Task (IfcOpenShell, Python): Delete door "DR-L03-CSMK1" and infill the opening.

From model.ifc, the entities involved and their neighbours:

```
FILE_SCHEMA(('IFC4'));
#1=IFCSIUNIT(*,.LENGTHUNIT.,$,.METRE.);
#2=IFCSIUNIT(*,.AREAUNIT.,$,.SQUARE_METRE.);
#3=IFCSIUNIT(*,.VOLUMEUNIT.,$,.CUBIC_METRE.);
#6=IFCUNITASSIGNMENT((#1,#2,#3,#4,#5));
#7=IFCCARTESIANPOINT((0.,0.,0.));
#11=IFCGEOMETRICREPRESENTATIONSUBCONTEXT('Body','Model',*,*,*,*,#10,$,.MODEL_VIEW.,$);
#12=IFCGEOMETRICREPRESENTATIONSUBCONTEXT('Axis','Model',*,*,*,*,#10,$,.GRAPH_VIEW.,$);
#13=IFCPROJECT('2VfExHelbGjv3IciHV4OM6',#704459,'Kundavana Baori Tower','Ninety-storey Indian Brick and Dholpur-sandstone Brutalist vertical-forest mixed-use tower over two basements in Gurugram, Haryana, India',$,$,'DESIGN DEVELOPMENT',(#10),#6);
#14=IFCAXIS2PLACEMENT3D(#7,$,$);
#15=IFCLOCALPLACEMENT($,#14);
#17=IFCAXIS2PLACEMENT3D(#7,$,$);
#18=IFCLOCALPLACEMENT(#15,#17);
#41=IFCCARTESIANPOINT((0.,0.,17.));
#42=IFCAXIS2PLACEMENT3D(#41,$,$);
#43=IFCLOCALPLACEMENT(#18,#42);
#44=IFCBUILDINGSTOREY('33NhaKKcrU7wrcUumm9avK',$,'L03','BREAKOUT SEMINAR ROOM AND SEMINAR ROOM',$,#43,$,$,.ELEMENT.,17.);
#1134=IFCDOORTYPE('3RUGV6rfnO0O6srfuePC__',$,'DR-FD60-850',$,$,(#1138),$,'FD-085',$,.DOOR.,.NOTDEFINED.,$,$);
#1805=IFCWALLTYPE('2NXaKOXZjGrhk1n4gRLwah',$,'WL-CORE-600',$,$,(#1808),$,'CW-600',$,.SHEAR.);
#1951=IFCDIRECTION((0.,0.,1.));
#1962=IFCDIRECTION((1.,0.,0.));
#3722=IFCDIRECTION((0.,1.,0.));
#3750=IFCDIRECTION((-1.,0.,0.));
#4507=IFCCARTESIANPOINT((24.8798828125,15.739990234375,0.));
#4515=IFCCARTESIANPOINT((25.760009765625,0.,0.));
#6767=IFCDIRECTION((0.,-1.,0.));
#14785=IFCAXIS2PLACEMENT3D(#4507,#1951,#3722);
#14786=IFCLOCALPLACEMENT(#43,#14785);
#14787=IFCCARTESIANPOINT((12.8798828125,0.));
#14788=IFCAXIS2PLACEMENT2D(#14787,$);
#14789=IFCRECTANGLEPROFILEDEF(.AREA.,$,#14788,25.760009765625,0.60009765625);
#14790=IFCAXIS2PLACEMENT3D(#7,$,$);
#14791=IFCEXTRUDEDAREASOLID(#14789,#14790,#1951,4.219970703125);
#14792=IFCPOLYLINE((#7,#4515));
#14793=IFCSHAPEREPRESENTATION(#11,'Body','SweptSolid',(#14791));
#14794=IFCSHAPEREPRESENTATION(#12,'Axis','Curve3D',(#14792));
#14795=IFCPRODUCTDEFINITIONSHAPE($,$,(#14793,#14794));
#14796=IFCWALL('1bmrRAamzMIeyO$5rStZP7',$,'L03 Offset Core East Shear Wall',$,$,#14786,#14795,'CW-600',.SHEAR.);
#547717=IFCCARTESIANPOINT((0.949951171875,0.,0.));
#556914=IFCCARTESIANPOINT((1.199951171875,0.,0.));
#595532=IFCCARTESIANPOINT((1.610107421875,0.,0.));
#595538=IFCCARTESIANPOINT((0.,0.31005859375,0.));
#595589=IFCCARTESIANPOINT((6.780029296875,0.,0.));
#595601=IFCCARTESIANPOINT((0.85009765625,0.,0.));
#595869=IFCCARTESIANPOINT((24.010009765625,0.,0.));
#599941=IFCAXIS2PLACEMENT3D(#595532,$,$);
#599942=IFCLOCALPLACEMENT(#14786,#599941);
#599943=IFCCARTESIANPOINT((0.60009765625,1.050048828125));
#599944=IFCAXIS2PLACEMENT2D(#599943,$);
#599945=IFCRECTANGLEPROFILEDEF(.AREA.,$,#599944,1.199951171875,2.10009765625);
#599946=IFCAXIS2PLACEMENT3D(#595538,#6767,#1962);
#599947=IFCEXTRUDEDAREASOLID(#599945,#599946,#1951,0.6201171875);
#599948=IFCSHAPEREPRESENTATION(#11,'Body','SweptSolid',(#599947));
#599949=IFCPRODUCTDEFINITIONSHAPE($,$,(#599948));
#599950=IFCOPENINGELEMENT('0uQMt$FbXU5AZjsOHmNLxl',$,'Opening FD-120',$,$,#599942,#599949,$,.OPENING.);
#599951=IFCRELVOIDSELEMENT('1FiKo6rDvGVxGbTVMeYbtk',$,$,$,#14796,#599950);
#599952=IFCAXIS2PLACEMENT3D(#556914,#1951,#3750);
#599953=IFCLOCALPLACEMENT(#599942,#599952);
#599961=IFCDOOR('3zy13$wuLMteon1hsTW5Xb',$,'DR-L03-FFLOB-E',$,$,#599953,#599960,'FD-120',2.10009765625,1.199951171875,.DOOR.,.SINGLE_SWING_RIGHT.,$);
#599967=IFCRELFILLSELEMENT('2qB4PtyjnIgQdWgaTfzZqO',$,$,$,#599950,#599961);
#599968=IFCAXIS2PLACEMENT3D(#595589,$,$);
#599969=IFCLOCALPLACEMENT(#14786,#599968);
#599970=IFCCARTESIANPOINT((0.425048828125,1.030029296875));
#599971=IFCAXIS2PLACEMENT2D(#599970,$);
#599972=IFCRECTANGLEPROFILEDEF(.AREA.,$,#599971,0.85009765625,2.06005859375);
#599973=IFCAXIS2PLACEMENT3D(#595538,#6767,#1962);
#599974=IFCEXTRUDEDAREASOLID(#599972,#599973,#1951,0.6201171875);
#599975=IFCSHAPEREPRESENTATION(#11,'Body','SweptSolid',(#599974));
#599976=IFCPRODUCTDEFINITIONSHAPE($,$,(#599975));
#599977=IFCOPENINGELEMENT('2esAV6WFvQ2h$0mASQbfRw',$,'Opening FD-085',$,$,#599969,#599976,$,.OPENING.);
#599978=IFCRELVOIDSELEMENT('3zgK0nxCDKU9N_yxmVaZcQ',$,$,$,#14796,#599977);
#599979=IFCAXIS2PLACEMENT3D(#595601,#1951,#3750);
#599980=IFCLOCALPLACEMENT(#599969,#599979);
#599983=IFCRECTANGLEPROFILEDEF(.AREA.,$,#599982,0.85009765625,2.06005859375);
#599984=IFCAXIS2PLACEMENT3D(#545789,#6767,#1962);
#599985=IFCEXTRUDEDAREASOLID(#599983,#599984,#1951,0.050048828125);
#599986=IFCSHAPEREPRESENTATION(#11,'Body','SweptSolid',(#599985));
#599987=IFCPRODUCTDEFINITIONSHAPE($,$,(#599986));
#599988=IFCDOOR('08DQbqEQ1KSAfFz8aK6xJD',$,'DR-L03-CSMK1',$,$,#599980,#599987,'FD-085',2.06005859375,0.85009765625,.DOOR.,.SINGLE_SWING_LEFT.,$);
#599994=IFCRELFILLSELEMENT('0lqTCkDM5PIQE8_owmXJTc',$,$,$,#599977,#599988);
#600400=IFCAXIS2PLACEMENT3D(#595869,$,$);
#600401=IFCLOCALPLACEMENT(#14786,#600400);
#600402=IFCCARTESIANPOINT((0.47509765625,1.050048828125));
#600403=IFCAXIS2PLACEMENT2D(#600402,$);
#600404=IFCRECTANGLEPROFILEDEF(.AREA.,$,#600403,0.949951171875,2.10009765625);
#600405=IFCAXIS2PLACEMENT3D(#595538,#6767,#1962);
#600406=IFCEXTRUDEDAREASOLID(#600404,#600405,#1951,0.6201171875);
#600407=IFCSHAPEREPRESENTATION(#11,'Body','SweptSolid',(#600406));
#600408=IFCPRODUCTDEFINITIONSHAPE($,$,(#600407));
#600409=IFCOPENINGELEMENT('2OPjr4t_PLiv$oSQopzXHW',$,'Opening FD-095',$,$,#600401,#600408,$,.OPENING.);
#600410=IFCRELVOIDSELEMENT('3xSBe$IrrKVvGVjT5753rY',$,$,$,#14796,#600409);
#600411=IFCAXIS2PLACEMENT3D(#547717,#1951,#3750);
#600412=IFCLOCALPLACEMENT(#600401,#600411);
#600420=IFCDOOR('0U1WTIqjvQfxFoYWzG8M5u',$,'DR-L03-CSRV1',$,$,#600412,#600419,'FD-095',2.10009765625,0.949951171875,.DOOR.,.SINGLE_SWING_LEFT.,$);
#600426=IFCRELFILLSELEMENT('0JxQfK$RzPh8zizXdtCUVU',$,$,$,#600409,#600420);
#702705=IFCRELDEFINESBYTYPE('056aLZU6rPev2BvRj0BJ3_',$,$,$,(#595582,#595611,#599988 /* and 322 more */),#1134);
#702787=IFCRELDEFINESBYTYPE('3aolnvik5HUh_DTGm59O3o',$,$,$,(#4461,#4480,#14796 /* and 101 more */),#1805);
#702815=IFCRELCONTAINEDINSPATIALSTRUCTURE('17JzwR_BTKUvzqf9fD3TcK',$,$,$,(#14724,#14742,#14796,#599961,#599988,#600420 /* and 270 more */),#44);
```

```python
import ifcopenshell
import ifcopenshell.api.feature
import ifcopenshell.api.root
import ifcopenshell.geom
import ifcopenshell.util.shape

model = ifcopenshell.open("model.ifc")
settings = ifcopenshell.geom.settings()


def volume(element):
    """Net volume in cubic metres, openings subtracted."""
    shape = ifcopenshell.geom.create_shape(settings, element)
    return ifcopenshell.util.shape.get_volume(shape.geometry)


door = model.by_guid("08DQbqEQ1KSAfFz8aK6xJD")
opening = door.FillsVoids[0].RelatingOpeningElement
wall = opening.VoidsElements[0].RelatingBuildingElement
before = volume(wall)

ifcopenshell.api.root.remove_product(model, product=door)
ifcopenshell.api.feature.remove_feature(model, feature=opening)

after = volume(wall)

print(f"wall volume {before:.3f} -> {after:.3f} m3")

model.write("model_edited.ifc")
```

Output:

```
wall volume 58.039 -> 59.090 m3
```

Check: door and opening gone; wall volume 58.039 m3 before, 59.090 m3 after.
